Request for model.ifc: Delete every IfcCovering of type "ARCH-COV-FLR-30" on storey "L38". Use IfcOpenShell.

First a look at what the model holds.

```python
import ifcopenshell
import ifcopenshell.util.element

model = ifcopenshell.open("model.ifc")
print(model.schema)
storey = next(s for s in model.by_type("IfcBuildingStorey") if s.Name == "L38")
coverings = [e for e in ifcopenshell.util.element.get_decomposition(storey) if e.is_a("IfcCovering")]
seen = {}
for e in coverings:
    element_type = ifcopenshell.util.element.get_type(e)
    name = element_type.Name if element_type not in (None, e) else None
    seen[name] = seen.get(name, 0) + 1
for name, count in sorted(seen.items(), key=str):
    print(count, "x", name)
```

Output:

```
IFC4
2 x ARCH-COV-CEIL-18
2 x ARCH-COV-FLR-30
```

```python
import ifcopenshell
import ifcopenshell.api.root
import ifcopenshell.util.element

model = ifcopenshell.open("model.ifc")

storey = next(s for s in model.by_type("IfcBuildingStorey") if s.Name == "L38")
coverings = [e for e in ifcopenshell.util.element.get_decomposition(storey) if e.is_a("IfcCovering")]
targets = [e for e in coverings if (t := ifcopenshell.util.element.get_type(e)) not in (None, e) and t.Name == "ARCH-COV-FLR-30"]

for e in targets:
    ifcopenshell.api.root.remove_product(model, product=e)
print(len(targets), "removed")

model.write("model_rev.ifc")
```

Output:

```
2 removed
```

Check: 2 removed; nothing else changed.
